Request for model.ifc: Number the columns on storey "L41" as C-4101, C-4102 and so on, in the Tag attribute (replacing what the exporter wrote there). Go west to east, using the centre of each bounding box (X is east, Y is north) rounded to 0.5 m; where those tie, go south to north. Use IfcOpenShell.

First a look at what the model holds.

```python
import ifcopenshell
import ifcopenshell.util.element
import ifcopenshell.util.placement

model = ifcopenshell.open("model.ifc")
print(model.schema)
storey = next(s for s in model.by_type("IfcBuildingStorey") if s.Name == "L41")
columns = [e for e in ifcopenshell.util.element.get_decomposition(storey) if e.is_a("IfcColumn")]
for e in sorted(columns, key=lambda e: e.id()):
    origin = ifcopenshell.util.placement.get_local_placement(e.ObjectPlacement)[:3, 3]
    print(e.id(), e.Tag, e.Name, origin.round(2) + 0.0, sep=" | ")
```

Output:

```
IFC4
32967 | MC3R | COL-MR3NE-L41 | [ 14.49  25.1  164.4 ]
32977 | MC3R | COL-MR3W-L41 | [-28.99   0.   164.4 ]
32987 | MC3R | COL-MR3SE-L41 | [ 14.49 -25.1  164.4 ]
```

```python
import ifcopenshell
import ifcopenshell.geom
import ifcopenshell.util.element
import ifcopenshell.util.shape

model = ifcopenshell.open("model.ifc")
settings = ifcopenshell.geom.settings()
settings.set("use-world-coords", True)


def centre(element):
    shape = ifcopenshell.geom.create_shape(settings, element)
    return ifcopenshell.util.shape.get_bbox_centroid(shape.geometry)


storey = next(s for s in model.by_type("IfcBuildingStorey") if s.Name == "L41")
columns = [e for e in ifcopenshell.util.element.get_decomposition(storey) if e.is_a("IfcColumn")]

# Insertion points can sit at a corner or the storey origin, so sort by the geometry (in metres).
centres = {e: centre(e) for e in columns}
columns.sort(key=lambda e: (round(centres[e][0] / 0.5), centres[e][1]))

for i, e in enumerate(columns, start=1):
    number = f"C-41{i:02d}"
    e.Tag = number
    print(e.id(), number)

model.write("model_v2.ifc")
```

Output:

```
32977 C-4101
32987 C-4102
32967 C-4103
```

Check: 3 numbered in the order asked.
